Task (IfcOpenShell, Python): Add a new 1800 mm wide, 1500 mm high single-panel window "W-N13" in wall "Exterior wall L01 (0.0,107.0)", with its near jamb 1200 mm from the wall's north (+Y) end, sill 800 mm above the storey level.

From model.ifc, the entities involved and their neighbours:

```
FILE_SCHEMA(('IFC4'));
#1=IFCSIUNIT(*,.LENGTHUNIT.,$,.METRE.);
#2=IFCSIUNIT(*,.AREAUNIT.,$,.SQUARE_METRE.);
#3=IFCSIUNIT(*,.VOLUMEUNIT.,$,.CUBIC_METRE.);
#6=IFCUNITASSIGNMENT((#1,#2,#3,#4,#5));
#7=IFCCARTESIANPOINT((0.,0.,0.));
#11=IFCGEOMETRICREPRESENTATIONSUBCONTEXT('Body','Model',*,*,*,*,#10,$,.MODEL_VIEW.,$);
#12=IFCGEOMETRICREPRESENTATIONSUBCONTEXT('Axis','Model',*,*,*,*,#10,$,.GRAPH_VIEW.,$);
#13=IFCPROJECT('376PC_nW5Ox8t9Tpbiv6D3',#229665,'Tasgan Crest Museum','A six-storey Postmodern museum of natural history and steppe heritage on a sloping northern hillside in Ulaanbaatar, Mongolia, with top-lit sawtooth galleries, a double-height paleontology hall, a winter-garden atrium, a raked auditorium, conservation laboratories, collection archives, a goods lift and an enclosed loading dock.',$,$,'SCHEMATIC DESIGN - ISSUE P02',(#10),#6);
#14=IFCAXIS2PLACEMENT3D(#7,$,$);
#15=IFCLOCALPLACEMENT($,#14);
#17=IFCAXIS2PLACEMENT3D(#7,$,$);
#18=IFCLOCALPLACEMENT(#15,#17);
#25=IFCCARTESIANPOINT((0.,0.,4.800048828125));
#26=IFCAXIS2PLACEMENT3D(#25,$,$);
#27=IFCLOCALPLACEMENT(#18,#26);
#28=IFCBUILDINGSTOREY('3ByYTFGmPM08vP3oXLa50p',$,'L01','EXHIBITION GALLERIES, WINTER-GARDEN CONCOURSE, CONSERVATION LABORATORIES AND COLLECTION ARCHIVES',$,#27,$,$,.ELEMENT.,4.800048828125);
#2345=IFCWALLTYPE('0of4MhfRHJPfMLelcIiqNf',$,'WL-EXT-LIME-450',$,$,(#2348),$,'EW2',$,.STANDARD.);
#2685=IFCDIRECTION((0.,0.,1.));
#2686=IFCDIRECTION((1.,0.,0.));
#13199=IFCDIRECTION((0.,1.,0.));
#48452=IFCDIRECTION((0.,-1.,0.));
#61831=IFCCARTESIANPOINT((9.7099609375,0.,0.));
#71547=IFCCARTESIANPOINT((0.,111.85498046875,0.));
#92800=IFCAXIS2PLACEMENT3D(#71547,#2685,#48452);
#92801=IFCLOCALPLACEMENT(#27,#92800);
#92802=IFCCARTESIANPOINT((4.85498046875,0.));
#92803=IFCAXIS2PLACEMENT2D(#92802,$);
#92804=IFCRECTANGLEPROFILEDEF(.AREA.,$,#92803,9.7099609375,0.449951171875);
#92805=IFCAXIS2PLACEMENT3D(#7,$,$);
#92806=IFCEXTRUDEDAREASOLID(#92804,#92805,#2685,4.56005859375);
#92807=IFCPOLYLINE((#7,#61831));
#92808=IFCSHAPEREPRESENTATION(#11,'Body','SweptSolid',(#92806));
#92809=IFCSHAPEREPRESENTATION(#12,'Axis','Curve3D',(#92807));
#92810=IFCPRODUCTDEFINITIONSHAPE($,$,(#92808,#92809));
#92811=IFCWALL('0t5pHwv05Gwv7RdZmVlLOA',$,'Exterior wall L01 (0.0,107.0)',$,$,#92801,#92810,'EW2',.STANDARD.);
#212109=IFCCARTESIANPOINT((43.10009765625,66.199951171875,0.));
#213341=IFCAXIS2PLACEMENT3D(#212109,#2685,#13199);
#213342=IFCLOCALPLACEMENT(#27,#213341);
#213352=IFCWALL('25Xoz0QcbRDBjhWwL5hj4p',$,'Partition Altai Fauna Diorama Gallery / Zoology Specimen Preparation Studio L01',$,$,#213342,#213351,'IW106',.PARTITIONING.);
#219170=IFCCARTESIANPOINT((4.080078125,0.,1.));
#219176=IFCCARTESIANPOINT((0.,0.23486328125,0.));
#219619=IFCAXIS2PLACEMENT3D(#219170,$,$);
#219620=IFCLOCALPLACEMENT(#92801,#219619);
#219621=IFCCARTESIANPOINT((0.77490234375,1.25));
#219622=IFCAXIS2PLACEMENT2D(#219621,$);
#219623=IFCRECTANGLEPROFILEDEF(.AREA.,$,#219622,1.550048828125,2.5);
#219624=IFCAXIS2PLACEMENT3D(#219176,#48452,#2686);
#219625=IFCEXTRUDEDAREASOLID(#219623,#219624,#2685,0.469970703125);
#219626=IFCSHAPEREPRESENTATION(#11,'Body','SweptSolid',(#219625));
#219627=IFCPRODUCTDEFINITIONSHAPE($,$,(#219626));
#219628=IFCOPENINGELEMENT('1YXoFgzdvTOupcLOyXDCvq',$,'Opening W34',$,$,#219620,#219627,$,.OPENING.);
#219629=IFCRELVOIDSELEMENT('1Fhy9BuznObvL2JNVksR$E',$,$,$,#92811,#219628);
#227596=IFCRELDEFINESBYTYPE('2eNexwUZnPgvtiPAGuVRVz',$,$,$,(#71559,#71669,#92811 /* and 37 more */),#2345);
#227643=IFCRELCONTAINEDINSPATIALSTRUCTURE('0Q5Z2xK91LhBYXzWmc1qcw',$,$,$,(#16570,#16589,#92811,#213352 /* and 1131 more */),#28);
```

```python
import numpy as np
import ifcopenshell
import ifcopenshell.api.feature
import ifcopenshell.api.geometry
import ifcopenshell.api.root
import ifcopenshell.api.spatial
import ifcopenshell.geom
import ifcopenshell.util.element
import ifcopenshell.util.placement
import ifcopenshell.util.representation
import ifcopenshell.util.shape
import ifcopenshell.util.unit

model = ifcopenshell.open("model.ifc")
unit_scale = ifcopenshell.util.unit.calculate_unit_scale(model)
settings = ifcopenshell.geom.settings()


def volume(element):
    """Net volume in cubic metres, openings subtracted."""
    shape = ifcopenshell.geom.create_shape(settings, element)
    return ifcopenshell.util.shape.get_volume(shape.geometry)


wall = model.by_id(92811)
storey = ifcopenshell.util.element.get_container(wall, ifc_class="IfcBuildingStorey")
context = ifcopenshell.util.representation.get_context(model, "Model", "Body", "MODEL_VIEW")
before = volume(wall)

width, height, from_end, sill = 1.8, 1.5, 1.2, 0.8  # metres

# The wall runs along its own X axis, and the end named is its -X end.
wall_shape = ifcopenshell.geom.create_shape(settings, wall)
x, y, z = ifcopenshell.util.shape.get_vertices(wall_shape.geometry).T
start = x.min() + from_end
face, thickness = float(y.min()), float(y.max() - y.min())
wall_matrix = ifcopenshell.util.placement.get_local_placement(wall.ObjectPlacement)
level = ifcopenshell.util.placement.get_local_placement(storey.ObjectPlacement)[2, 3]


def in_wall(x, y):
    """Placement at x, y metres in the wall's axes, at sill height."""
    matrix = wall_matrix.copy()
    matrix[:, 3] = wall_matrix @ np.array([x / unit_scale, y / unit_scale, 0.0, 1.0])
    matrix[2, 3] = level + sill / unit_scale
    return matrix


# Opening: a box that overshoots both wall faces by 50 mm.
opening = ifcopenshell.api.root.create_entity(model, ifc_class="IfcOpeningElement", predefined_type="OPENING")
box = ifcopenshell.api.geometry.add_wall_representation(
    model, context=context, length=width, height=height, thickness=thickness + 0.1
)
ifcopenshell.api.geometry.assign_representation(model, product=opening, representation=box)
ifcopenshell.api.geometry.edit_object_placement(model, product=opening, matrix=in_wall(start, face - 0.05), is_si=False)
ifcopenshell.api.feature.add_feature(model, feature=opening, element=wall)

window = ifcopenshell.api.root.create_entity(model, ifc_class="IfcWindow", name="W-N13", predefined_type="WINDOW")
window.OverallWidth, window.OverallHeight = width / unit_scale, height / unit_scale
window.PartitioningType = "SINGLE_PANEL"
body = ifcopenshell.api.geometry.add_window_representation(
    model,
    context=context,
    overall_width=window.OverallWidth,
    overall_height=window.OverallHeight,
    partition_type="SINGLE_PANEL",
)
ifcopenshell.api.geometry.assign_representation(model, product=window, representation=body)
ifcopenshell.api.spatial.assign_container(model, products=[window], relating_structure=storey)
ifcopenshell.api.feature.add_filling(model, opening=opening, element=window)

# Centre the window in the wall's thickness.
ifcopenshell.api.geometry.edit_object_placement(model, product=window, matrix=in_wall(start, face), is_si=False)
window_shape = ifcopenshell.geom.create_shape(settings, window)
depth = ifcopenshell.util.shape.get_vertices(window_shape.geometry)[:, 1]
offset = face + thickness / 2 - (depth.min() + depth.max()) / 2
ifcopenshell.api.geometry.edit_object_placement(model, product=window, matrix=in_wall(start, offset), is_si=False)

after = volume(wall)

print(f"wall volume {before:.3f} -> {after:.3f} m3")

model.write("model_edited.ifc")
```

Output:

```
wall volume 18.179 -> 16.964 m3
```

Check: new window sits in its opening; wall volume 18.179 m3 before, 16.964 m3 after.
